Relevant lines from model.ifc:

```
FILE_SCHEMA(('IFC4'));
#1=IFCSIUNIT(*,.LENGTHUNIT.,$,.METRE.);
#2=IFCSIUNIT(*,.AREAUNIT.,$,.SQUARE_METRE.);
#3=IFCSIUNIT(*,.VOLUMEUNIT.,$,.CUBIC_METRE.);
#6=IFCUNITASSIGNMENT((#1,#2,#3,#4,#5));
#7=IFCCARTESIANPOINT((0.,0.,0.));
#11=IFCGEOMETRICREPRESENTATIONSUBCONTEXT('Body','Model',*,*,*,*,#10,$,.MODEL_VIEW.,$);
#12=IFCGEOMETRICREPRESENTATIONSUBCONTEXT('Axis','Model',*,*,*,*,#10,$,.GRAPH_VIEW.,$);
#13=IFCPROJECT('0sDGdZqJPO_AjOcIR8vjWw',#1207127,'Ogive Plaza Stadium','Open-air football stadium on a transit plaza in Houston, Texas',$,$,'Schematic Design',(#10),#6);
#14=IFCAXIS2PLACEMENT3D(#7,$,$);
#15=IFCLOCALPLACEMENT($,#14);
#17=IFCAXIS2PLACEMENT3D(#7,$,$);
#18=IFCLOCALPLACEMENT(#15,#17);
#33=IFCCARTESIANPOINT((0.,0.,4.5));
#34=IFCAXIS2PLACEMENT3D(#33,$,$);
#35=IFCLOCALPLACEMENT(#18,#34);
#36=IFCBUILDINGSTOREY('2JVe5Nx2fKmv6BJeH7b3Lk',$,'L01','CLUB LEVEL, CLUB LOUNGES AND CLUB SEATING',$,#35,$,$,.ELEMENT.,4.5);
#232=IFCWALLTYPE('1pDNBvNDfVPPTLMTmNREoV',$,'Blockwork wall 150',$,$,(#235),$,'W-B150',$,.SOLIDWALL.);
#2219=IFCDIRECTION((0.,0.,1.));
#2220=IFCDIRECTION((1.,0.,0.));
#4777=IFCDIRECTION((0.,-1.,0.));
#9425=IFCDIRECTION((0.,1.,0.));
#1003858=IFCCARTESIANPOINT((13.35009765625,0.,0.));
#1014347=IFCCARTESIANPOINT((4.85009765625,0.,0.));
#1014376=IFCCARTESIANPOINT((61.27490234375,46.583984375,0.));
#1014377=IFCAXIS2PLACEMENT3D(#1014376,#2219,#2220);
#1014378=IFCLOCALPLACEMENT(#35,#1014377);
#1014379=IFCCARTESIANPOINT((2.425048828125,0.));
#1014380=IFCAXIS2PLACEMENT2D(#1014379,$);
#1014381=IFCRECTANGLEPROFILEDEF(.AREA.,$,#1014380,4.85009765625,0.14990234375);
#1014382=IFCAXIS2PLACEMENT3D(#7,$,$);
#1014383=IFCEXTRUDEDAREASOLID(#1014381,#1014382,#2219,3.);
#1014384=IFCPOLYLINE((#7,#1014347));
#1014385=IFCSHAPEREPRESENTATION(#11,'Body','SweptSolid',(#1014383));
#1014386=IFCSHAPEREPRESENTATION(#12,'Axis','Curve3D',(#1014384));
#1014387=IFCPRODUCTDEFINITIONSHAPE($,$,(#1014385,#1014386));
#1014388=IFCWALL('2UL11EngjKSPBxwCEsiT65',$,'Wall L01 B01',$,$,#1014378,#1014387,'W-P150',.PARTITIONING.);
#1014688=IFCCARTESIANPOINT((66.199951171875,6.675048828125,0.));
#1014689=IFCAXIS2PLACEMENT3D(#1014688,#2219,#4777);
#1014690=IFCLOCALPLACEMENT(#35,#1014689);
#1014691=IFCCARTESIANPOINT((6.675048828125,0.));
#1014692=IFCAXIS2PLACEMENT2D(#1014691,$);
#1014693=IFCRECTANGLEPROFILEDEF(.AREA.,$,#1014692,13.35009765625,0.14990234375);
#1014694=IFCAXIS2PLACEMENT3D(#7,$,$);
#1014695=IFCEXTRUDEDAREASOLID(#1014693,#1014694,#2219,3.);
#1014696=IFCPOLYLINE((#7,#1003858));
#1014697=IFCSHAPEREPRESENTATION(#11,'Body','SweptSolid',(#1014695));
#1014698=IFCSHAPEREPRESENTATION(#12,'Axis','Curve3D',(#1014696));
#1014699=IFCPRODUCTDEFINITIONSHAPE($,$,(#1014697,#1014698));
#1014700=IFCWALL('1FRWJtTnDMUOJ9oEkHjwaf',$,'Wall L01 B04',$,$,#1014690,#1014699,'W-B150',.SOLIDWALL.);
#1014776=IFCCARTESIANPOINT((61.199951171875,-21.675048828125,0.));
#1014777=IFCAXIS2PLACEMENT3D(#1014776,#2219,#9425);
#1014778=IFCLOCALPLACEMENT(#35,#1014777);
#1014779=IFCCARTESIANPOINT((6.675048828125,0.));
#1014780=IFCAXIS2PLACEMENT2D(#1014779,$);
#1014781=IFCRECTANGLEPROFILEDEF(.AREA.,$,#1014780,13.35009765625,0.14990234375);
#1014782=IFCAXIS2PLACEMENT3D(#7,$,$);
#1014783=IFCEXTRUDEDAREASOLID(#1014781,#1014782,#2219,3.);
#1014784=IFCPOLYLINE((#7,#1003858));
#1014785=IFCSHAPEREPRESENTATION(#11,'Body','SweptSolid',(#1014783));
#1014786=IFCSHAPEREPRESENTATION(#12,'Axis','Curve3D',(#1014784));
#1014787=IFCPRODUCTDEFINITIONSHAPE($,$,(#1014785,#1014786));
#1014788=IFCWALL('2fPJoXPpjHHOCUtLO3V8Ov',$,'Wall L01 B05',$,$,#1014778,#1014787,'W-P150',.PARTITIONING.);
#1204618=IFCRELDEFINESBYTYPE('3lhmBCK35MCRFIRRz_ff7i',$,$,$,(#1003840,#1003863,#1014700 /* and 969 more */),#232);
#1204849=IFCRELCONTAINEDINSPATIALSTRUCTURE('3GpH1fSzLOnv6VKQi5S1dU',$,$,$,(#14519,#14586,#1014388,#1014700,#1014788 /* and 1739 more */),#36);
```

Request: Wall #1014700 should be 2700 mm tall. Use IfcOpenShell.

```python
import ifcopenshell
import ifcopenshell.geom
import ifcopenshell.util.representation
import ifcopenshell.util.shape
import ifcopenshell.util.unit

model = ifcopenshell.open("model.ifc")
unit_scale = ifcopenshell.util.unit.calculate_unit_scale(model)
settings = ifcopenshell.geom.settings()


def volume(element):
    """Net volume in cubic metres, openings subtracted."""
    shape = ifcopenshell.geom.create_shape(settings, element)
    return ifcopenshell.util.shape.get_volume(shape.geometry)


wall = model.by_guid("1FRWJtTnDMUOJ9oEkHjwaf")
before = volume(wall)

body = ifcopenshell.util.representation.get_representation(wall, "Model", "Body")
solid = body.Items[0]
old_height = solid.Depth
solid.Depth = 2.7 / unit_scale
after = volume(wall)

print(f"height {old_height:g} -> {solid.Depth:g}, volume {before:.3f} -> {after:.3f} m3")

model.write("model_updated.ifc")
```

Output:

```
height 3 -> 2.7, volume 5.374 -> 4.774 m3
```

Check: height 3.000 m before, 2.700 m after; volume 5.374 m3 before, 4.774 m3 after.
